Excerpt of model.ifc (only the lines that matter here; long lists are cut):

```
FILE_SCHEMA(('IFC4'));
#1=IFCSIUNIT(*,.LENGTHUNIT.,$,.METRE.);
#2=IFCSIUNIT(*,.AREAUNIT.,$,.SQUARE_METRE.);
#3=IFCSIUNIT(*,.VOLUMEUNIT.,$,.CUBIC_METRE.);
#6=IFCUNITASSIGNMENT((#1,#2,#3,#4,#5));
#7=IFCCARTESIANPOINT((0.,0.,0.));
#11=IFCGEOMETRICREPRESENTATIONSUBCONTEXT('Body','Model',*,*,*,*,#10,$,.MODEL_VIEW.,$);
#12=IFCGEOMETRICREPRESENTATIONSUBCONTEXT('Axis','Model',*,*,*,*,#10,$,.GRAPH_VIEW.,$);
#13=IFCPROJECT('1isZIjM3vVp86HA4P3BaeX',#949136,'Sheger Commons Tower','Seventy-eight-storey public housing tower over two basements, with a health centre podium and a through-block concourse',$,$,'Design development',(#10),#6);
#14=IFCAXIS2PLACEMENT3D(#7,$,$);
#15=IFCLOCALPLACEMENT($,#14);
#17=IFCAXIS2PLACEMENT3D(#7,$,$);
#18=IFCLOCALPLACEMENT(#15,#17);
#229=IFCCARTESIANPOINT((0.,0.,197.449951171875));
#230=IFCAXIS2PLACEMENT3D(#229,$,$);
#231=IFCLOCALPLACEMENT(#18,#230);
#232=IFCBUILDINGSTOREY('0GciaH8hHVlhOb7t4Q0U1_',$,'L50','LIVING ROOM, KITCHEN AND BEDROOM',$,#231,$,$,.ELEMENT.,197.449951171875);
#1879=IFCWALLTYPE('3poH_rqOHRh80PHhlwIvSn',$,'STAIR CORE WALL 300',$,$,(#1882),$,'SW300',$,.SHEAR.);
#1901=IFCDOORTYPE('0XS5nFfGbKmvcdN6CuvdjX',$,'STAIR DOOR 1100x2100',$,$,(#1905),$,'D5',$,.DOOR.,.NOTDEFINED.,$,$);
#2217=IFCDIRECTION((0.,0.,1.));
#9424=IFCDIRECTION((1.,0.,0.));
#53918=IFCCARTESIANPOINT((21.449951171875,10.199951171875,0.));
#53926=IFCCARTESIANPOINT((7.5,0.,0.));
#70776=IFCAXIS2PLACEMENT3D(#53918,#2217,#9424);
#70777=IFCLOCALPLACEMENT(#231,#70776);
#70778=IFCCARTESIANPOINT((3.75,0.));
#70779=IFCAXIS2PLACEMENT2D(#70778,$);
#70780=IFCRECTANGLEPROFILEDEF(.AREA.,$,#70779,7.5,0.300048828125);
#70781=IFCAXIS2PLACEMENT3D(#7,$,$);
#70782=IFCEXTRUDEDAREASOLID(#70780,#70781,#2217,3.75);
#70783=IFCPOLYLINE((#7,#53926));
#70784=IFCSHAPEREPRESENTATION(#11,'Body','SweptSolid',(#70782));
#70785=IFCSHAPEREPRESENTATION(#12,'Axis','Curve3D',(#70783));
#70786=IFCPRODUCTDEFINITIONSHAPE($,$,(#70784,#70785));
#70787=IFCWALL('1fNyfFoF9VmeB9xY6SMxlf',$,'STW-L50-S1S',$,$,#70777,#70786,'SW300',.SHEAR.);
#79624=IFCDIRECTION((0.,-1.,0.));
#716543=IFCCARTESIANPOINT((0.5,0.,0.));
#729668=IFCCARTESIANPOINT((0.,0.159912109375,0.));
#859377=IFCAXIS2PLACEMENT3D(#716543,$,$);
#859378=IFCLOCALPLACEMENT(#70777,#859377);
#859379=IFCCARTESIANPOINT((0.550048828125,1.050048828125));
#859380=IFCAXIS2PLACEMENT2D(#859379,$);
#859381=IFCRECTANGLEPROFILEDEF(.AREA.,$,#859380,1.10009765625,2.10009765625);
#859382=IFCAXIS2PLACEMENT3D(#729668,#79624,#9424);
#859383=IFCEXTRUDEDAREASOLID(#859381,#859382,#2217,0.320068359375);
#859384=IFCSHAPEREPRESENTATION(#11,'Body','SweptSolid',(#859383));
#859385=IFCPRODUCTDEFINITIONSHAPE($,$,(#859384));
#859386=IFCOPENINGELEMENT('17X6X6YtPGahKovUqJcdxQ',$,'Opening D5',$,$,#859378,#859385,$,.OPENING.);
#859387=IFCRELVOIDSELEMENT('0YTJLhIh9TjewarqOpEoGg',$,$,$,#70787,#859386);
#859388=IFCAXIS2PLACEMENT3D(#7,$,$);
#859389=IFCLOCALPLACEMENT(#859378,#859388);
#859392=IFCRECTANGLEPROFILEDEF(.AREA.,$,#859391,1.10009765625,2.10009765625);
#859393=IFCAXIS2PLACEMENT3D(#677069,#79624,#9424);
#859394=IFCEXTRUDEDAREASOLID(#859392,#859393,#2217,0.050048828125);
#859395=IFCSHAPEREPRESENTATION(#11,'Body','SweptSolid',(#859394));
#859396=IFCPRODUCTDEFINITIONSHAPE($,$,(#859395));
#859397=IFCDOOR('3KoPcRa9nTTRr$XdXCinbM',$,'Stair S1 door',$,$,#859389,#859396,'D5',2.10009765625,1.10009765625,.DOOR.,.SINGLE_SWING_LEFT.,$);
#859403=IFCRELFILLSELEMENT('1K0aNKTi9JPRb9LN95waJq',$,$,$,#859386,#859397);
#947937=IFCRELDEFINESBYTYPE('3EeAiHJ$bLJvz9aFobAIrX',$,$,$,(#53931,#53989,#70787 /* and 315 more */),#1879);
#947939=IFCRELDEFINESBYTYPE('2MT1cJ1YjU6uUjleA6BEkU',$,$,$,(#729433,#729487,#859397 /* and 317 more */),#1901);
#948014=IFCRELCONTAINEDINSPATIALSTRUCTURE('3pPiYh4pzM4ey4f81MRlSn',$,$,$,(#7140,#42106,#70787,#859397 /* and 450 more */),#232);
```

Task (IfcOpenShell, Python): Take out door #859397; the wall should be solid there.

```python
import ifcopenshell
import ifcopenshell.api.feature
import ifcopenshell.api.root
import ifcopenshell.geom
import ifcopenshell.util.shape

model = ifcopenshell.open("model.ifc")
settings = ifcopenshell.geom.settings()


def volume(element):
    """Net volume in cubic metres, openings subtracted."""
    shape = ifcopenshell.geom.create_shape(settings, element)
    return ifcopenshell.util.shape.get_volume(shape.geometry)


door = model.by_guid("3KoPcRa9nTTRr$XdXCinbM")
opening = door.FillsVoids[0].RelatingOpeningElement
wall = opening.VoidsElements[0].RelatingBuildingElement
before = volume(wall)

ifcopenshell.api.root.remove_product(model, product=door)
ifcopenshell.api.feature.remove_feature(model, feature=opening)

after = volume(wall)

print(f"wall volume {before:.3f} -> {after:.3f} m3")

model.write("model-out.ifc")
```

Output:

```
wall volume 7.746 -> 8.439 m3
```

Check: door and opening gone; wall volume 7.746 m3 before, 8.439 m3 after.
